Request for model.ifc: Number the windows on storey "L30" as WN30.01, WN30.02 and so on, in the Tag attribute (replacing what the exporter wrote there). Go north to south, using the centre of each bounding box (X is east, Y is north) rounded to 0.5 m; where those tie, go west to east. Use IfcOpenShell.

First a look at what the model holds.

```python
import ifcopenshell
import ifcopenshell.util.element
import ifcopenshell.util.placement

model = ifcopenshell.open("model.ifc")
print(model.schema)
storey = next(s for s in model.by_type("IfcBuildingStorey") if s.Name == "L30")
windows = [e for e in ifcopenshell.util.element.get_decomposition(storey) if e.is_a("IfcWindow")]
for e in sorted(windows, key=lambda e: e.id()):
    origin = ifcopenshell.util.placement.get_local_placement(e.ObjectPlacement)[:3, 3]
    print(e.id(), e.Tag, e.Name, origin.round(2) + 0.0, sep=" | ")
```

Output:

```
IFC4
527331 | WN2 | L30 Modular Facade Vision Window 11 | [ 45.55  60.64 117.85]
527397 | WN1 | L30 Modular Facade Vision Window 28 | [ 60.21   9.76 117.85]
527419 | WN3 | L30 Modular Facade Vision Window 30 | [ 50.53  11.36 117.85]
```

```python
import ifcopenshell
import ifcopenshell.geom
import ifcopenshell.util.element
import ifcopenshell.util.shape

model = ifcopenshell.open("model.ifc")
settings = ifcopenshell.geom.settings()
settings.set("use-world-coords", True)


def centre(element):
    shape = ifcopenshell.geom.create_shape(settings, element)
    return ifcopenshell.util.shape.get_bbox_centroid(shape.geometry)


storey = next(s for s in model.by_type("IfcBuildingStorey") if s.Name == "L30")
windows = [e for e in ifcopenshell.util.element.get_decomposition(storey) if e.is_a("IfcWindow")]

# Insertion points can sit at a corner or the storey origin, so sort by the geometry (in metres).
centres = {e: centre(e) for e in windows}
windows.sort(key=lambda e: (-round(centres[e][1] / 0.5), centres[e][0]))

for i, e in enumerate(windows, start=1):
    number = f"WN30.{i:02d}"
    e.Tag = number
    print(e.id(), number)

model.write("model_v2.ifc")
```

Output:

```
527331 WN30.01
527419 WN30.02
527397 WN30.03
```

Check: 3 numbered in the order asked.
